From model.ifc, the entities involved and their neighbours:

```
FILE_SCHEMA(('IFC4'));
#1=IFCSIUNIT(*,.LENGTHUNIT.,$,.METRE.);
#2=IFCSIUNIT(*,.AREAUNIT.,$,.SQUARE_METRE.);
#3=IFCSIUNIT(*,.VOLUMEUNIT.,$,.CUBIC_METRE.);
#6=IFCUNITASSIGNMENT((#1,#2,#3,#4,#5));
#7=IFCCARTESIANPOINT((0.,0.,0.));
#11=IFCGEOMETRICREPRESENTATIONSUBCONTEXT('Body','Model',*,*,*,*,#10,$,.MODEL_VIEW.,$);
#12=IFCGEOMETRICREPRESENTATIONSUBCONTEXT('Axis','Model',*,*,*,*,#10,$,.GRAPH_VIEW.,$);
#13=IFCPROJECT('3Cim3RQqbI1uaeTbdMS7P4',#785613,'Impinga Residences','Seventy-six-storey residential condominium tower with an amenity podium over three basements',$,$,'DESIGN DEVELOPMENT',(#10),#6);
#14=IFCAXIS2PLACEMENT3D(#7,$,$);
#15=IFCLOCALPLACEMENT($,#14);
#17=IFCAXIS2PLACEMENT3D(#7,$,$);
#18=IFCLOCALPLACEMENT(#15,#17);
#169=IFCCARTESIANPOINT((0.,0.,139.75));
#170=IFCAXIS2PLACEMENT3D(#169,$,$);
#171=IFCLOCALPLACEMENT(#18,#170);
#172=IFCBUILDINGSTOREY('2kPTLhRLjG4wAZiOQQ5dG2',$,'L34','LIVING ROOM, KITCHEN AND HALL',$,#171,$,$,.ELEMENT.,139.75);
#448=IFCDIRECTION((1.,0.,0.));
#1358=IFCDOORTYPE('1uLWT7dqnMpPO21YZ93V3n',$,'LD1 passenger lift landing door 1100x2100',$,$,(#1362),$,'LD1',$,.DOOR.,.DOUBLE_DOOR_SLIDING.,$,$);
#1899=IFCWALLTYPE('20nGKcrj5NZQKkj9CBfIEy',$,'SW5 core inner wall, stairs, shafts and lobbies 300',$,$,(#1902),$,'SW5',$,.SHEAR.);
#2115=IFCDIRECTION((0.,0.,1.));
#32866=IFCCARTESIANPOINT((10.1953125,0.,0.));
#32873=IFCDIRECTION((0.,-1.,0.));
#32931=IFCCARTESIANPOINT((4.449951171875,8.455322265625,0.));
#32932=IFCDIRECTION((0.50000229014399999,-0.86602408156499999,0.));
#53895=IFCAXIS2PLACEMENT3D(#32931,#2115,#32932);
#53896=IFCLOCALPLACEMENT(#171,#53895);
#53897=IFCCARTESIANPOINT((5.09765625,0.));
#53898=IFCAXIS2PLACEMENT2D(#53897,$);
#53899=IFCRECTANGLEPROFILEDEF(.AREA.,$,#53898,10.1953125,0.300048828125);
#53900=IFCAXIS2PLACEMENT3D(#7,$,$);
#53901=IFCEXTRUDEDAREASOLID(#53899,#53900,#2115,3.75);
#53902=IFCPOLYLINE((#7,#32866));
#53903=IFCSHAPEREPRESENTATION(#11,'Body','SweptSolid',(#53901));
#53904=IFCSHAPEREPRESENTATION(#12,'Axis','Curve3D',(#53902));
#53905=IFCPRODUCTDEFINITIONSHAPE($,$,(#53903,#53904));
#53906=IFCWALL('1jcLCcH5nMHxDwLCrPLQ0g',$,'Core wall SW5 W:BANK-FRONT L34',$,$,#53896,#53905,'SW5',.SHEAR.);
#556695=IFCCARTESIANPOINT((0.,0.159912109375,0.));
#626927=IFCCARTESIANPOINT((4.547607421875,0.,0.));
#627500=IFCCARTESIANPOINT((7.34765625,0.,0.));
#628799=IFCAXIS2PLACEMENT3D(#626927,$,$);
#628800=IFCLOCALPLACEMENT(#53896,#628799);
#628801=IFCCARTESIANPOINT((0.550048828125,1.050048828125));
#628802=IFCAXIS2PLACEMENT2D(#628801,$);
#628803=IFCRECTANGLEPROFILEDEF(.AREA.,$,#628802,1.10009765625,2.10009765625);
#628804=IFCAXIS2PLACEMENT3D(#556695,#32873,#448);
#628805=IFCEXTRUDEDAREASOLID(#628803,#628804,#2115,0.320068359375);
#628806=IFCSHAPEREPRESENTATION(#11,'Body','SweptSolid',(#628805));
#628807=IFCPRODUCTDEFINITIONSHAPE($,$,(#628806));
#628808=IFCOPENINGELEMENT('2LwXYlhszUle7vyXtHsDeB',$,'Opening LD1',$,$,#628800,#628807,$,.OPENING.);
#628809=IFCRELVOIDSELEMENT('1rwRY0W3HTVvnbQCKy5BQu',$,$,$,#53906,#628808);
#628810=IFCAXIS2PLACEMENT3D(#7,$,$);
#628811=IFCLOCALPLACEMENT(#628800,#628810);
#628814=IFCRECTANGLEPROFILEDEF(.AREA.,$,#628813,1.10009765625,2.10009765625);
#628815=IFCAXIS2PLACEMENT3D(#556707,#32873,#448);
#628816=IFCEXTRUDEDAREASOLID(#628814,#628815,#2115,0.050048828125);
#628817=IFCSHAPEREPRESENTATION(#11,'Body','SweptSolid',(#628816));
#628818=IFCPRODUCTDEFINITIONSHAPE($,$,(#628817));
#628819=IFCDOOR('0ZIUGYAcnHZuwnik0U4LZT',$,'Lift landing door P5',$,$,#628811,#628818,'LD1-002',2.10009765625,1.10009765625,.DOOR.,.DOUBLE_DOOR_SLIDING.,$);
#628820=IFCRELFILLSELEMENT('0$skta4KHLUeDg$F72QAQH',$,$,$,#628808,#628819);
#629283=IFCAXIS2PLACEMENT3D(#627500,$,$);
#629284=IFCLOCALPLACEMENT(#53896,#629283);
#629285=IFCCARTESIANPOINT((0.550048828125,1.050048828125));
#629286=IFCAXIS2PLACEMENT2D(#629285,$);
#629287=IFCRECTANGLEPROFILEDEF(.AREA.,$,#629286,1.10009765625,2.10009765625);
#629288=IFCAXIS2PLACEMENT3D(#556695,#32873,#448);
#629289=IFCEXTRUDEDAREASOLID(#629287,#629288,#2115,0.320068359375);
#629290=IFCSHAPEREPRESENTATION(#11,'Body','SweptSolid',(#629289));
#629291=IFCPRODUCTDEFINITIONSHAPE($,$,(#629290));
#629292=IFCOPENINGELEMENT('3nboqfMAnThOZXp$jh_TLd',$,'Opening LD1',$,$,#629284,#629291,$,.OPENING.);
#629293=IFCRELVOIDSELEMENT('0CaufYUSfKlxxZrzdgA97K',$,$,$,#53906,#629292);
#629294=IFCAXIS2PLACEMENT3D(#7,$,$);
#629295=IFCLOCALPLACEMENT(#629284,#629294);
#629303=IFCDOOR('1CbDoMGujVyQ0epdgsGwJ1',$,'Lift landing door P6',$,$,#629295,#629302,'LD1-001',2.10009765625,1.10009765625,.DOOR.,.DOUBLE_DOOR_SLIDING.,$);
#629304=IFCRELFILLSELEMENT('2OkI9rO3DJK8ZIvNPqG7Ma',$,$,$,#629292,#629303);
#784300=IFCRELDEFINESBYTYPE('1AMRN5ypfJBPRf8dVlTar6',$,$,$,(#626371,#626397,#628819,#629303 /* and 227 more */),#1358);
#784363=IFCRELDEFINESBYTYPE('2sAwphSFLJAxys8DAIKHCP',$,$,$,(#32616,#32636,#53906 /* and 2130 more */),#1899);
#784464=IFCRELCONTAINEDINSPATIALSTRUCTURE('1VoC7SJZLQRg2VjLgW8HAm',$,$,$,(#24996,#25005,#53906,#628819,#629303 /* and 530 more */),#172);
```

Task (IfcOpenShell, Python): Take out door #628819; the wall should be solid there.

```python
import ifcopenshell
import ifcopenshell.api.feature
import ifcopenshell.api.root
import ifcopenshell.geom
import ifcopenshell.util.shape

model = ifcopenshell.open("model.ifc")
settings = ifcopenshell.geom.settings()


def volume(element):
    """Net volume in cubic metres, openings subtracted."""
    shape = ifcopenshell.geom.create_shape(settings, element)
    return ifcopenshell.util.shape.get_volume(shape.geometry)


door = model.by_guid("0ZIUGYAcnHZuwnik0U4LZT")
opening = door.FillsVoids[0].RelatingOpeningElement
wall = opening.VoidsElements[0].RelatingBuildingElement
before = volume(wall)

ifcopenshell.api.root.remove_product(model, product=door)
ifcopenshell.api.feature.remove_feature(model, feature=opening)

after = volume(wall)

print(f"wall volume {before:.3f} -> {after:.3f} m3")

model.write("model_updated.ifc")
```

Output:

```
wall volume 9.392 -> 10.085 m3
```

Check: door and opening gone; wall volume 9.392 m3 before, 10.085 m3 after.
